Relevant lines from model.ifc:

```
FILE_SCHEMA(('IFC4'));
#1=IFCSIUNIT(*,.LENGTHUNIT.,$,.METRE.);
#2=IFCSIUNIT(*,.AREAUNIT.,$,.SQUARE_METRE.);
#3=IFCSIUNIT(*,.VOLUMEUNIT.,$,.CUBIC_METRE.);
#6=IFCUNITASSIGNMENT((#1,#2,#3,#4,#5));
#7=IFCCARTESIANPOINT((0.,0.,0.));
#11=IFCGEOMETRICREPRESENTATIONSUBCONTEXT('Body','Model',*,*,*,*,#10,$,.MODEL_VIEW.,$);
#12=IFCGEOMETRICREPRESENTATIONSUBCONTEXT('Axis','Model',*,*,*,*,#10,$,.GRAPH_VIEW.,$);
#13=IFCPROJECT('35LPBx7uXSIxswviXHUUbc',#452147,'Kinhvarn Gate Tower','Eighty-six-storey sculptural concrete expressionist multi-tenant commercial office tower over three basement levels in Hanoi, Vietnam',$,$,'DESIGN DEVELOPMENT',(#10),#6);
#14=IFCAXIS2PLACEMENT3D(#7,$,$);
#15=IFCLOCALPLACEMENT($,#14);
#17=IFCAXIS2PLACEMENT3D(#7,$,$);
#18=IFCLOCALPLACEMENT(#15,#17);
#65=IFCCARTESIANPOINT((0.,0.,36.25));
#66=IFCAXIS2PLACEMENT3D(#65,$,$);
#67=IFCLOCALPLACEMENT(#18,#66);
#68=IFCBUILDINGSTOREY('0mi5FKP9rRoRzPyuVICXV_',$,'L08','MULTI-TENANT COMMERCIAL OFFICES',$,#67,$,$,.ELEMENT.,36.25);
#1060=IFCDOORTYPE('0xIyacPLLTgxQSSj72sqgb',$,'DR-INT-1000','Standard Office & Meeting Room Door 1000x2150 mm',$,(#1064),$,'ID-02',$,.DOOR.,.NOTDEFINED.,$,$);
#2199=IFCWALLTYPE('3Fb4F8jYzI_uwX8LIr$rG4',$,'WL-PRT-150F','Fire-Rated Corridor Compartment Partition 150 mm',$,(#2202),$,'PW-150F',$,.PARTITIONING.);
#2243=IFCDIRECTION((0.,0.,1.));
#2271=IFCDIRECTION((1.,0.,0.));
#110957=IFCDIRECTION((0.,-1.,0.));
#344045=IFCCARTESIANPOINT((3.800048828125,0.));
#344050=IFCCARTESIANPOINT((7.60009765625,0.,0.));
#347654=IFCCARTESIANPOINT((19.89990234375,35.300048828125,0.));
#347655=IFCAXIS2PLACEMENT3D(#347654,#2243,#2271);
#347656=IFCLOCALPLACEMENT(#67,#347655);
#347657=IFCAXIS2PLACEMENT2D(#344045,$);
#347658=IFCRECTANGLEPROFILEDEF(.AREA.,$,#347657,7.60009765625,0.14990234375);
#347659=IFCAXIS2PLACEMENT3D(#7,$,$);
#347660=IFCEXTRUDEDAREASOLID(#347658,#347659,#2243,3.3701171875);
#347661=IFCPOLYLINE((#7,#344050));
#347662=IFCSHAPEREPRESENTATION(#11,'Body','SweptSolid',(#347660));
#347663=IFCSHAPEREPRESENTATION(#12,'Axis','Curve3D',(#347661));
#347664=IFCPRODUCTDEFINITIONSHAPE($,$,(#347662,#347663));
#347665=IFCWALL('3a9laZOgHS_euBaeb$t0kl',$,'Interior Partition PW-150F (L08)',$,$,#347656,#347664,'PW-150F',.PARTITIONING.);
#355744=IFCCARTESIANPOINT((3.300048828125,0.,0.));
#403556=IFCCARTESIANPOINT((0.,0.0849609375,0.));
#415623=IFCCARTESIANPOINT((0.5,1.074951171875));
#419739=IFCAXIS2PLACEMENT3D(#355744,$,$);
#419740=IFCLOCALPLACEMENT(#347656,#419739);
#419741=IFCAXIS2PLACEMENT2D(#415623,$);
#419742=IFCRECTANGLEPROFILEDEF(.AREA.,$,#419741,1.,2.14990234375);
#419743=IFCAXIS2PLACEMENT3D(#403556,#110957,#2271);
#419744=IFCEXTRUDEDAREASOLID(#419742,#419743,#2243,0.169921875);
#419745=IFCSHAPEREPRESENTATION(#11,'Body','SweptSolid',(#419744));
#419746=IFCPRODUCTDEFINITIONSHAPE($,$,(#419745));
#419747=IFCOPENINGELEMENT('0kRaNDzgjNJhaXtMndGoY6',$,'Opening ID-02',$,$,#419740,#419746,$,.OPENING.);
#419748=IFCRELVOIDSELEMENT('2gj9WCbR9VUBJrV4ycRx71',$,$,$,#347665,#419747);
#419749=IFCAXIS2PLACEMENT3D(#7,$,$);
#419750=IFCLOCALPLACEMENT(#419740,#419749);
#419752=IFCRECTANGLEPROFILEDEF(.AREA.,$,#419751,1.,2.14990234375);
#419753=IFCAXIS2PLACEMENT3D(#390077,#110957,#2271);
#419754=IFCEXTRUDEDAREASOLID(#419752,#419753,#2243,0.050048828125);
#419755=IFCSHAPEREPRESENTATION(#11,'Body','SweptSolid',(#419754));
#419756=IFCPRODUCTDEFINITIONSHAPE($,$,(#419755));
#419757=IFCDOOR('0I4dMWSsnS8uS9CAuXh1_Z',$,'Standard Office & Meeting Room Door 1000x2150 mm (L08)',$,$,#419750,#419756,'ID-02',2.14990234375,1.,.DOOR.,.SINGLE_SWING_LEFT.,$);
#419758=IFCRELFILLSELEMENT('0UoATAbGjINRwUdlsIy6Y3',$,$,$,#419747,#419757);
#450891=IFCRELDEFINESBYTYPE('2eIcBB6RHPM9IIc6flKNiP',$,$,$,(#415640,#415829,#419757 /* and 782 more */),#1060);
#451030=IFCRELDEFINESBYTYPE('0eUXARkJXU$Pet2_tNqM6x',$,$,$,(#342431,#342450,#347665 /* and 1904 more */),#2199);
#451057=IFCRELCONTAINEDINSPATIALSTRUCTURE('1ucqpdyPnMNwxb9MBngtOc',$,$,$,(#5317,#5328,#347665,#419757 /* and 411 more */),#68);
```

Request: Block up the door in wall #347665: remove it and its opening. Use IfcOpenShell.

```python
import ifcopenshell
import ifcopenshell.api.feature
import ifcopenshell.api.root
import ifcopenshell.geom
import ifcopenshell.util.shape

model = ifcopenshell.open("model.ifc")
settings = ifcopenshell.geom.settings()


def volume(element):
    """Net volume in cubic metres, openings subtracted."""
    shape = ifcopenshell.geom.create_shape(settings, element)
    return ifcopenshell.util.shape.get_volume(shape.geometry)


door = model.by_id(419757)
opening = door.FillsVoids[0].RelatingOpeningElement
wall = opening.VoidsElements[0].RelatingBuildingElement
before = volume(wall)

ifcopenshell.api.root.remove_product(model, product=door)
ifcopenshell.api.feature.remove_feature(model, feature=opening)

after = volume(wall)

print(f"wall volume {before:.3f} -> {after:.3f} m3")

model.write("model_v2.ifc")
```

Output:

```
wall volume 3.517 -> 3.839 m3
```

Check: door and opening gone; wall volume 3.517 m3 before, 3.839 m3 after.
